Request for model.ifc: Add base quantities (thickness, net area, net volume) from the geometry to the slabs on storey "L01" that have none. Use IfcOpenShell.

First a look at what the model holds.

```python
import ifcopenshell
import ifcopenshell.util.element
import ifcopenshell.util.unit

model = ifcopenshell.open("model.ifc")
print(model.schema)
for unit_type in ("LENGTHUNIT", "AREAUNIT", "VOLUMEUNIT"):
    print(unit_type, ifcopenshell.util.unit.calculate_unit_scale(model, unit_type))
storey = next(s for s in model.by_type("IfcBuildingStorey") if s.Name == "L01")
slabs = [e for e in ifcopenshell.util.element.get_decomposition(storey) if e.is_a("IfcSlab")]
for e in sorted(slabs, key=lambda e: e.id()):
    print(e.id(), e.is_a(), e.Name, list(ifcopenshell.util.element.get_psets(e, qtos_only=True)), sep=" | ")
```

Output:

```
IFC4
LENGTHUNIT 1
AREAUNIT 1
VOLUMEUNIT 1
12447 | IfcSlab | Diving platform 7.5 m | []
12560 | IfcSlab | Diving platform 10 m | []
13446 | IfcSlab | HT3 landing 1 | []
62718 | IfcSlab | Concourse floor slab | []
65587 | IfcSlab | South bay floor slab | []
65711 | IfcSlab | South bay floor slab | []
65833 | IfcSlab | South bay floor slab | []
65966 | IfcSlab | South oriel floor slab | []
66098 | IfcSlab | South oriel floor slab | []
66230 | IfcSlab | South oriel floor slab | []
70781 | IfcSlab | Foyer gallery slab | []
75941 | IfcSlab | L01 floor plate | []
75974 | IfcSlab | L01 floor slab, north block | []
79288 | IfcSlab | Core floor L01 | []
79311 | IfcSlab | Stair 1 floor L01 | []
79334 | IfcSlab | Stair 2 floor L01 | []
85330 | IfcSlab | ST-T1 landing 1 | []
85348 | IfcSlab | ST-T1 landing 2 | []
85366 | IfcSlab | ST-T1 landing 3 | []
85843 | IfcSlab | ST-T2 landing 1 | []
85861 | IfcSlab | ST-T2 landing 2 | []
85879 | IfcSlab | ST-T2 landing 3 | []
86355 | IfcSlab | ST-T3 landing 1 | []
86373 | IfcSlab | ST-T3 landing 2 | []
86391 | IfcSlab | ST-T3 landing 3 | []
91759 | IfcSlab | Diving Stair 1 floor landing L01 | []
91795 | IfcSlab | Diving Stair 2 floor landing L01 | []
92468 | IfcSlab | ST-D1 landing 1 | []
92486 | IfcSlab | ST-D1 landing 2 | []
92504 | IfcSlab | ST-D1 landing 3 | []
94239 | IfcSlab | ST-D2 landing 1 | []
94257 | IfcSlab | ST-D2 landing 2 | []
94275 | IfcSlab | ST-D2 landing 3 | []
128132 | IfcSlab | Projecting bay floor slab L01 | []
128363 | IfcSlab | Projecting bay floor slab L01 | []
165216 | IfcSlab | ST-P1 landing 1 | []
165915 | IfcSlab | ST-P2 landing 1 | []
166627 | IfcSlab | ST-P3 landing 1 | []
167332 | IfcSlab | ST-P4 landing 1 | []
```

```python
import ifcopenshell
import ifcopenshell.api.pset
import ifcopenshell.geom
import ifcopenshell.util.element
import ifcopenshell.util.shape
import ifcopenshell.util.unit

model = ifcopenshell.open("model.ifc")
unit_scale = ifcopenshell.util.unit.calculate_unit_scale(model)
area_scale = ifcopenshell.util.unit.calculate_unit_scale(model, "AREAUNIT")
volume_scale = ifcopenshell.util.unit.calculate_unit_scale(model, "VOLUMEUNIT")
settings = ifcopenshell.geom.settings()

storey = next(s for s in model.by_type("IfcBuildingStorey") if s.Name == "L01")
slabs = [e for e in ifcopenshell.util.element.get_decomposition(storey) if e.is_a("IfcSlab")]

for e in sorted(slabs, key=lambda e: e.id()):
    if ifcopenshell.util.element.get_psets(e, qtos_only=True, should_inherit=False):
        continue
    # Geometry comes back in metres, in the element's own axes.
    shape = ifcopenshell.geom.create_shape(settings, e)
    values = {
        "Width": ifcopenshell.util.shape.get_z(shape.geometry) / unit_scale,
        "NetArea": ifcopenshell.util.shape.get_footprint_area(shape.geometry) / area_scale,
        "NetVolume": ifcopenshell.util.shape.get_volume(shape.geometry) / volume_scale,
    }
    qto = ifcopenshell.api.pset.add_qto(model, product=e, name="Qto_SlabBaseQuantities")
    ifcopenshell.api.pset.edit_qto(model, qto=qto, properties=values)
    print(e.id(), {k: round(v, 3) for k, v in values.items()})

model.write("model_edited.ifc")
```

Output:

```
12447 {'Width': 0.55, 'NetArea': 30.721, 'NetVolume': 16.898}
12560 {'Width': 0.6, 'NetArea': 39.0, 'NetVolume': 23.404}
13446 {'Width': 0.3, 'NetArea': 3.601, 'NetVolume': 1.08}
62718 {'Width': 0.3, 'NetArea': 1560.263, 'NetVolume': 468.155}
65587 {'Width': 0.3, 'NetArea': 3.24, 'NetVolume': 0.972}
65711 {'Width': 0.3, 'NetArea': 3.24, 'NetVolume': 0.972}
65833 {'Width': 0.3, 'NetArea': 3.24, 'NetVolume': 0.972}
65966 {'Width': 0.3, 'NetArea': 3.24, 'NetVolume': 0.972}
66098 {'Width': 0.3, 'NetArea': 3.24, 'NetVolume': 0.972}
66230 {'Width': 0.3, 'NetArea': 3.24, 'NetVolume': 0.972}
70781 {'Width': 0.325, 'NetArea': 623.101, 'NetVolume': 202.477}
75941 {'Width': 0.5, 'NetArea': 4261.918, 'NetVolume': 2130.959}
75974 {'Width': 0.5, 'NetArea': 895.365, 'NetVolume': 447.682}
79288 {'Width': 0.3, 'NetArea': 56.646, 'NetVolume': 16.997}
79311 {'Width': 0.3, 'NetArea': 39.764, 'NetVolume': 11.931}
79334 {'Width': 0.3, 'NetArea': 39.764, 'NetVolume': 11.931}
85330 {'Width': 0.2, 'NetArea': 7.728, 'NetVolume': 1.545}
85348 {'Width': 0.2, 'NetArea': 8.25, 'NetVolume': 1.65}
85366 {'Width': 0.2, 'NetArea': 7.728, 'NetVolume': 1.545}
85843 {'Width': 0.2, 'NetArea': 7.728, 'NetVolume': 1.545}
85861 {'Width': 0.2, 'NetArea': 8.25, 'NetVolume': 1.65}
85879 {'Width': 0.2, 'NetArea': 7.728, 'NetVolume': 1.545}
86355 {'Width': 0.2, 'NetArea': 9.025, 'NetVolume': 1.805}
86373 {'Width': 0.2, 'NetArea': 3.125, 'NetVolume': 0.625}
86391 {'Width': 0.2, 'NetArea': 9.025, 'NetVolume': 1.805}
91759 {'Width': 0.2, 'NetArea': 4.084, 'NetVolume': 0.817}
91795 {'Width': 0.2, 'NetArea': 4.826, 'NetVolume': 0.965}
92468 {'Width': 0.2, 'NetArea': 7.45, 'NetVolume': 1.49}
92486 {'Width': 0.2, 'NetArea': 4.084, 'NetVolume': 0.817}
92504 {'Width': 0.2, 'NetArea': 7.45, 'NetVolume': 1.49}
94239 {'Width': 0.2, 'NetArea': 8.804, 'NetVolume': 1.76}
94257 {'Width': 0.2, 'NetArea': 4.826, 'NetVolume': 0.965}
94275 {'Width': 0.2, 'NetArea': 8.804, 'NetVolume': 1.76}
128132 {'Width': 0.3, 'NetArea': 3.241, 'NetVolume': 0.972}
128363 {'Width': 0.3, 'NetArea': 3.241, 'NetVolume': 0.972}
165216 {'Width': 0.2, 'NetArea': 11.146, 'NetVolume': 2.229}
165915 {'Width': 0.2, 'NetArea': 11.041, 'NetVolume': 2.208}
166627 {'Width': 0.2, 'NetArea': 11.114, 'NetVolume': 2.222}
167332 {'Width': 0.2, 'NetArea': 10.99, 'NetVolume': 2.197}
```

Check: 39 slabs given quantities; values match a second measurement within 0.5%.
